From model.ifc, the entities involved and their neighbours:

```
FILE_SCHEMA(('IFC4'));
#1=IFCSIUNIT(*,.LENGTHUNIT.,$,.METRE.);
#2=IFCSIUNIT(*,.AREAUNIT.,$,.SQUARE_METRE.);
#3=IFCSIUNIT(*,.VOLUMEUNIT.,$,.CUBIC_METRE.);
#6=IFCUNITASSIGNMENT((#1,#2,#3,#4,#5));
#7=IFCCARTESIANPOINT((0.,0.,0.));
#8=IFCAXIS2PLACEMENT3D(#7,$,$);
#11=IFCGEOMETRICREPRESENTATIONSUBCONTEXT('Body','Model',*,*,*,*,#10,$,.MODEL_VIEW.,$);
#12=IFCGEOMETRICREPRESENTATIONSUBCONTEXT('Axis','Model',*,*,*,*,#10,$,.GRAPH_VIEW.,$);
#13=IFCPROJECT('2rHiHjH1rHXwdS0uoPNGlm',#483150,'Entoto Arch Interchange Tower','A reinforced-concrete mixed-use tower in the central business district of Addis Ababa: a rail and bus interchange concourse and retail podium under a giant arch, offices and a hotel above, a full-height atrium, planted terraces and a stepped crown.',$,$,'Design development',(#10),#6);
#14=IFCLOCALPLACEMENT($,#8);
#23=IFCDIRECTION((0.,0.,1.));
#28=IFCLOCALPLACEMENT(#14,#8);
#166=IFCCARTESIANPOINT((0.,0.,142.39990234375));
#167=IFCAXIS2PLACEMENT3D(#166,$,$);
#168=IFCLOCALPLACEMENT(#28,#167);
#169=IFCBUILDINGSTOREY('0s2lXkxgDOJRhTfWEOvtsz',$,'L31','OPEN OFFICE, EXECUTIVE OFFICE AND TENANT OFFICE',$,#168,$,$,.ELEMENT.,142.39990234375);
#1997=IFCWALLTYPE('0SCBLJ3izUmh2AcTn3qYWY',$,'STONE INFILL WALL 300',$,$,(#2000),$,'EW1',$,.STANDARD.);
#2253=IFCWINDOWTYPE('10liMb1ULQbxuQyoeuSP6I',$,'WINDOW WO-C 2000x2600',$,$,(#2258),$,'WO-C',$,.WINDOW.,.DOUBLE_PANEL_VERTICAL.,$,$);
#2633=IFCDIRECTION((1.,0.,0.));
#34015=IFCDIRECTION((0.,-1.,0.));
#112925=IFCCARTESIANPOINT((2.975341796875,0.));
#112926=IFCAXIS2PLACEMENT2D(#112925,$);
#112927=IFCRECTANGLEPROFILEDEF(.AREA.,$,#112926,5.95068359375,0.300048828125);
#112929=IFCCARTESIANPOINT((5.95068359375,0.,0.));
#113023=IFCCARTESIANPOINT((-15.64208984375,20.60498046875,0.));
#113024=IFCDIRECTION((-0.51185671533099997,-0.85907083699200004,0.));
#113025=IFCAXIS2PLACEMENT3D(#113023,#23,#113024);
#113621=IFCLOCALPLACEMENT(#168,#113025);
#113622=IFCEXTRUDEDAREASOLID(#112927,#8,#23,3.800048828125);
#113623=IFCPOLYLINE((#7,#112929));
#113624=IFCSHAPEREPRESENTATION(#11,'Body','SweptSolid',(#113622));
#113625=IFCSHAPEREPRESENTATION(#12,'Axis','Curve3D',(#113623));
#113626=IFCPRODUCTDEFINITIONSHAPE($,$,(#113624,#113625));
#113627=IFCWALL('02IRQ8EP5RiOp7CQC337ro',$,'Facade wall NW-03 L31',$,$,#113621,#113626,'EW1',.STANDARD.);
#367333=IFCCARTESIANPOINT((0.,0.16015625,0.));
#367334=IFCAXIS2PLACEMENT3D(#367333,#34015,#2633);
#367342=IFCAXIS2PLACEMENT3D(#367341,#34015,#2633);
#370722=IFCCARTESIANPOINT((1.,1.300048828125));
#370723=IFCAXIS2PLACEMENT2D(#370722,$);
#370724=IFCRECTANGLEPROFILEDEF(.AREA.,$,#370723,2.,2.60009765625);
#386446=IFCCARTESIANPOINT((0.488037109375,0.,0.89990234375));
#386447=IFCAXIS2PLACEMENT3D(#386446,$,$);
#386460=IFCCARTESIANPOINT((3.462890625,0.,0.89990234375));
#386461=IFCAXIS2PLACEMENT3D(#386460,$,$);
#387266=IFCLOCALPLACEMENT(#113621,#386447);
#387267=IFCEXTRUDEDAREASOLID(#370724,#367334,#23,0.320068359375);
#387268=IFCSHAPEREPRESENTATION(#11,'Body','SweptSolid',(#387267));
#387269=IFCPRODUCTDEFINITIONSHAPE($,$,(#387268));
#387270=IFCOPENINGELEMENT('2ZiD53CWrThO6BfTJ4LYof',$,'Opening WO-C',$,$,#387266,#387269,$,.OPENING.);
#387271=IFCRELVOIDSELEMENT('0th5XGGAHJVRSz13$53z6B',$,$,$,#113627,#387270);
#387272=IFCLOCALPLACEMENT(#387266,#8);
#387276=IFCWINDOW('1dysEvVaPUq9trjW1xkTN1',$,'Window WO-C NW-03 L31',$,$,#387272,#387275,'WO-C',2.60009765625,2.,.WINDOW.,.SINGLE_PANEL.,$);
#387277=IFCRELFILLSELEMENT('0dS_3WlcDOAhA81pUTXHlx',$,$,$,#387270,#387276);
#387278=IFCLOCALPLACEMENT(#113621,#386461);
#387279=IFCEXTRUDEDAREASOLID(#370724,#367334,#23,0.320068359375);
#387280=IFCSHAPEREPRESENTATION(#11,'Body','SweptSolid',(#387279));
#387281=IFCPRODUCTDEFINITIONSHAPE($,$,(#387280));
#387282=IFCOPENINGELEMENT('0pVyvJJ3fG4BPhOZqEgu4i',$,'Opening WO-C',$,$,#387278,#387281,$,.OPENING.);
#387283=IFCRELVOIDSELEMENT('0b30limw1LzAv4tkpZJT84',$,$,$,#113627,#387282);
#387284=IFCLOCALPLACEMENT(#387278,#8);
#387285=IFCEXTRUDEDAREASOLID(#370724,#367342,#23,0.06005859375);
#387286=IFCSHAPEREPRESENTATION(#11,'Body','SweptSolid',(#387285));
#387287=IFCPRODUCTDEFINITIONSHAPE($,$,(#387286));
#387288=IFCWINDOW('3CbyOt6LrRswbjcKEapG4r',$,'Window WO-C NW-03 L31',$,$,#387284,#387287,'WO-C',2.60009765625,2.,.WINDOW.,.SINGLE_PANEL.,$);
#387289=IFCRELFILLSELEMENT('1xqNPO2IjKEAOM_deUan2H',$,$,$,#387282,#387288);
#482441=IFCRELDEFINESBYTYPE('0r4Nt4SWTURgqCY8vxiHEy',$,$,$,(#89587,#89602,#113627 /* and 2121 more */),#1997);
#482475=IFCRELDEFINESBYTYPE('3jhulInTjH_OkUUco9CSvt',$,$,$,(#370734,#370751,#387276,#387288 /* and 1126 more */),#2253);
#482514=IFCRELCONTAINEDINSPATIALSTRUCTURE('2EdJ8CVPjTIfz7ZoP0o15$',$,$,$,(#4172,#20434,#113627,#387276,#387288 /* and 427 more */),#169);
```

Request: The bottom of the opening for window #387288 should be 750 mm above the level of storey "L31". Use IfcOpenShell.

```python
import numpy as np
import ifcopenshell
import ifcopenshell.api.geometry
import ifcopenshell.geom
import ifcopenshell.util.element
import ifcopenshell.util.placement
import ifcopenshell.util.shape
import ifcopenshell.util.unit

model = ifcopenshell.open("model.ifc")
unit_scale = ifcopenshell.util.unit.calculate_unit_scale(model)

window = model.by_id(387288)
opening = window.FillsVoids[0].RelatingOpeningElement
storey = ifcopenshell.util.element.get_container(window, ifc_class="IfcBuildingStorey")
level = ifcopenshell.util.placement.get_local_placement(storey.ObjectPlacement)[2, 3]

# The opening's origin need not be at the sill, so measure its lowest point.
shape = ifcopenshell.geom.create_shape(ifcopenshell.geom.settings(), opening)
bottom = ifcopenshell.util.shape.get_shape_bottom_elevation(shape, shape.geometry) / unit_scale
dz = level + 0.75 / unit_scale - bottom

shift = np.array([0.0, 0.0, dz])
# The window is placed relative to its opening, so it follows when the opening moves.
matrix = ifcopenshell.util.placement.get_local_placement(opening.ObjectPlacement)
matrix[:3, 3] += shift
ifcopenshell.api.geometry.edit_object_placement(
    model, product=opening, matrix=matrix, is_si=False, should_transform_children=True
)

print(f"moved by {dz * unit_scale:+.3f} m")

model.write("model_edited.ifc")
```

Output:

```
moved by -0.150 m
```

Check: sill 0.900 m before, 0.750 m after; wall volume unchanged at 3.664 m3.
